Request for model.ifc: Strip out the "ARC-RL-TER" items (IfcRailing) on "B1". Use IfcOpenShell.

First a look at what the model holds.

```python
import ifcopenshell
import ifcopenshell.util.element

model = ifcopenshell.open("model.ifc")
print(model.schema)
storey = next(s for s in model.by_type("IfcBuildingStorey") if s.Name == "B1")
railings = [e for e in ifcopenshell.util.element.get_decomposition(storey) if e.is_a("IfcRailing")]
seen = {}
for e in railings:
    element_type = ifcopenshell.util.element.get_type(e)
    name = element_type.Name if element_type not in (None, e) else None
    seen[name] = seen.get(name, 0) + 1
for name, count in sorted(seen.items(), key=str):
    print(count, "x", name)
```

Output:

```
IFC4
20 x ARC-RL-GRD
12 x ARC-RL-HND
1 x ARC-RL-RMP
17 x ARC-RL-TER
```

```python
import ifcopenshell
import ifcopenshell.api.root
import ifcopenshell.util.element

model = ifcopenshell.open("model.ifc")

storey = next(s for s in model.by_type("IfcBuildingStorey") if s.Name == "B1")
railings = [e for e in ifcopenshell.util.element.get_decomposition(storey) if e.is_a("IfcRailing")]
targets = [e for e in railings if (t := ifcopenshell.util.element.get_type(e)) not in (None, e) and t.Name == "ARC-RL-TER"]

for e in targets:
    ifcopenshell.api.root.remove_product(model, product=e)
print(len(targets), "removed")

model.write("model_v2.ifc")
```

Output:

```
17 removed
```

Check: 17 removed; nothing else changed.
